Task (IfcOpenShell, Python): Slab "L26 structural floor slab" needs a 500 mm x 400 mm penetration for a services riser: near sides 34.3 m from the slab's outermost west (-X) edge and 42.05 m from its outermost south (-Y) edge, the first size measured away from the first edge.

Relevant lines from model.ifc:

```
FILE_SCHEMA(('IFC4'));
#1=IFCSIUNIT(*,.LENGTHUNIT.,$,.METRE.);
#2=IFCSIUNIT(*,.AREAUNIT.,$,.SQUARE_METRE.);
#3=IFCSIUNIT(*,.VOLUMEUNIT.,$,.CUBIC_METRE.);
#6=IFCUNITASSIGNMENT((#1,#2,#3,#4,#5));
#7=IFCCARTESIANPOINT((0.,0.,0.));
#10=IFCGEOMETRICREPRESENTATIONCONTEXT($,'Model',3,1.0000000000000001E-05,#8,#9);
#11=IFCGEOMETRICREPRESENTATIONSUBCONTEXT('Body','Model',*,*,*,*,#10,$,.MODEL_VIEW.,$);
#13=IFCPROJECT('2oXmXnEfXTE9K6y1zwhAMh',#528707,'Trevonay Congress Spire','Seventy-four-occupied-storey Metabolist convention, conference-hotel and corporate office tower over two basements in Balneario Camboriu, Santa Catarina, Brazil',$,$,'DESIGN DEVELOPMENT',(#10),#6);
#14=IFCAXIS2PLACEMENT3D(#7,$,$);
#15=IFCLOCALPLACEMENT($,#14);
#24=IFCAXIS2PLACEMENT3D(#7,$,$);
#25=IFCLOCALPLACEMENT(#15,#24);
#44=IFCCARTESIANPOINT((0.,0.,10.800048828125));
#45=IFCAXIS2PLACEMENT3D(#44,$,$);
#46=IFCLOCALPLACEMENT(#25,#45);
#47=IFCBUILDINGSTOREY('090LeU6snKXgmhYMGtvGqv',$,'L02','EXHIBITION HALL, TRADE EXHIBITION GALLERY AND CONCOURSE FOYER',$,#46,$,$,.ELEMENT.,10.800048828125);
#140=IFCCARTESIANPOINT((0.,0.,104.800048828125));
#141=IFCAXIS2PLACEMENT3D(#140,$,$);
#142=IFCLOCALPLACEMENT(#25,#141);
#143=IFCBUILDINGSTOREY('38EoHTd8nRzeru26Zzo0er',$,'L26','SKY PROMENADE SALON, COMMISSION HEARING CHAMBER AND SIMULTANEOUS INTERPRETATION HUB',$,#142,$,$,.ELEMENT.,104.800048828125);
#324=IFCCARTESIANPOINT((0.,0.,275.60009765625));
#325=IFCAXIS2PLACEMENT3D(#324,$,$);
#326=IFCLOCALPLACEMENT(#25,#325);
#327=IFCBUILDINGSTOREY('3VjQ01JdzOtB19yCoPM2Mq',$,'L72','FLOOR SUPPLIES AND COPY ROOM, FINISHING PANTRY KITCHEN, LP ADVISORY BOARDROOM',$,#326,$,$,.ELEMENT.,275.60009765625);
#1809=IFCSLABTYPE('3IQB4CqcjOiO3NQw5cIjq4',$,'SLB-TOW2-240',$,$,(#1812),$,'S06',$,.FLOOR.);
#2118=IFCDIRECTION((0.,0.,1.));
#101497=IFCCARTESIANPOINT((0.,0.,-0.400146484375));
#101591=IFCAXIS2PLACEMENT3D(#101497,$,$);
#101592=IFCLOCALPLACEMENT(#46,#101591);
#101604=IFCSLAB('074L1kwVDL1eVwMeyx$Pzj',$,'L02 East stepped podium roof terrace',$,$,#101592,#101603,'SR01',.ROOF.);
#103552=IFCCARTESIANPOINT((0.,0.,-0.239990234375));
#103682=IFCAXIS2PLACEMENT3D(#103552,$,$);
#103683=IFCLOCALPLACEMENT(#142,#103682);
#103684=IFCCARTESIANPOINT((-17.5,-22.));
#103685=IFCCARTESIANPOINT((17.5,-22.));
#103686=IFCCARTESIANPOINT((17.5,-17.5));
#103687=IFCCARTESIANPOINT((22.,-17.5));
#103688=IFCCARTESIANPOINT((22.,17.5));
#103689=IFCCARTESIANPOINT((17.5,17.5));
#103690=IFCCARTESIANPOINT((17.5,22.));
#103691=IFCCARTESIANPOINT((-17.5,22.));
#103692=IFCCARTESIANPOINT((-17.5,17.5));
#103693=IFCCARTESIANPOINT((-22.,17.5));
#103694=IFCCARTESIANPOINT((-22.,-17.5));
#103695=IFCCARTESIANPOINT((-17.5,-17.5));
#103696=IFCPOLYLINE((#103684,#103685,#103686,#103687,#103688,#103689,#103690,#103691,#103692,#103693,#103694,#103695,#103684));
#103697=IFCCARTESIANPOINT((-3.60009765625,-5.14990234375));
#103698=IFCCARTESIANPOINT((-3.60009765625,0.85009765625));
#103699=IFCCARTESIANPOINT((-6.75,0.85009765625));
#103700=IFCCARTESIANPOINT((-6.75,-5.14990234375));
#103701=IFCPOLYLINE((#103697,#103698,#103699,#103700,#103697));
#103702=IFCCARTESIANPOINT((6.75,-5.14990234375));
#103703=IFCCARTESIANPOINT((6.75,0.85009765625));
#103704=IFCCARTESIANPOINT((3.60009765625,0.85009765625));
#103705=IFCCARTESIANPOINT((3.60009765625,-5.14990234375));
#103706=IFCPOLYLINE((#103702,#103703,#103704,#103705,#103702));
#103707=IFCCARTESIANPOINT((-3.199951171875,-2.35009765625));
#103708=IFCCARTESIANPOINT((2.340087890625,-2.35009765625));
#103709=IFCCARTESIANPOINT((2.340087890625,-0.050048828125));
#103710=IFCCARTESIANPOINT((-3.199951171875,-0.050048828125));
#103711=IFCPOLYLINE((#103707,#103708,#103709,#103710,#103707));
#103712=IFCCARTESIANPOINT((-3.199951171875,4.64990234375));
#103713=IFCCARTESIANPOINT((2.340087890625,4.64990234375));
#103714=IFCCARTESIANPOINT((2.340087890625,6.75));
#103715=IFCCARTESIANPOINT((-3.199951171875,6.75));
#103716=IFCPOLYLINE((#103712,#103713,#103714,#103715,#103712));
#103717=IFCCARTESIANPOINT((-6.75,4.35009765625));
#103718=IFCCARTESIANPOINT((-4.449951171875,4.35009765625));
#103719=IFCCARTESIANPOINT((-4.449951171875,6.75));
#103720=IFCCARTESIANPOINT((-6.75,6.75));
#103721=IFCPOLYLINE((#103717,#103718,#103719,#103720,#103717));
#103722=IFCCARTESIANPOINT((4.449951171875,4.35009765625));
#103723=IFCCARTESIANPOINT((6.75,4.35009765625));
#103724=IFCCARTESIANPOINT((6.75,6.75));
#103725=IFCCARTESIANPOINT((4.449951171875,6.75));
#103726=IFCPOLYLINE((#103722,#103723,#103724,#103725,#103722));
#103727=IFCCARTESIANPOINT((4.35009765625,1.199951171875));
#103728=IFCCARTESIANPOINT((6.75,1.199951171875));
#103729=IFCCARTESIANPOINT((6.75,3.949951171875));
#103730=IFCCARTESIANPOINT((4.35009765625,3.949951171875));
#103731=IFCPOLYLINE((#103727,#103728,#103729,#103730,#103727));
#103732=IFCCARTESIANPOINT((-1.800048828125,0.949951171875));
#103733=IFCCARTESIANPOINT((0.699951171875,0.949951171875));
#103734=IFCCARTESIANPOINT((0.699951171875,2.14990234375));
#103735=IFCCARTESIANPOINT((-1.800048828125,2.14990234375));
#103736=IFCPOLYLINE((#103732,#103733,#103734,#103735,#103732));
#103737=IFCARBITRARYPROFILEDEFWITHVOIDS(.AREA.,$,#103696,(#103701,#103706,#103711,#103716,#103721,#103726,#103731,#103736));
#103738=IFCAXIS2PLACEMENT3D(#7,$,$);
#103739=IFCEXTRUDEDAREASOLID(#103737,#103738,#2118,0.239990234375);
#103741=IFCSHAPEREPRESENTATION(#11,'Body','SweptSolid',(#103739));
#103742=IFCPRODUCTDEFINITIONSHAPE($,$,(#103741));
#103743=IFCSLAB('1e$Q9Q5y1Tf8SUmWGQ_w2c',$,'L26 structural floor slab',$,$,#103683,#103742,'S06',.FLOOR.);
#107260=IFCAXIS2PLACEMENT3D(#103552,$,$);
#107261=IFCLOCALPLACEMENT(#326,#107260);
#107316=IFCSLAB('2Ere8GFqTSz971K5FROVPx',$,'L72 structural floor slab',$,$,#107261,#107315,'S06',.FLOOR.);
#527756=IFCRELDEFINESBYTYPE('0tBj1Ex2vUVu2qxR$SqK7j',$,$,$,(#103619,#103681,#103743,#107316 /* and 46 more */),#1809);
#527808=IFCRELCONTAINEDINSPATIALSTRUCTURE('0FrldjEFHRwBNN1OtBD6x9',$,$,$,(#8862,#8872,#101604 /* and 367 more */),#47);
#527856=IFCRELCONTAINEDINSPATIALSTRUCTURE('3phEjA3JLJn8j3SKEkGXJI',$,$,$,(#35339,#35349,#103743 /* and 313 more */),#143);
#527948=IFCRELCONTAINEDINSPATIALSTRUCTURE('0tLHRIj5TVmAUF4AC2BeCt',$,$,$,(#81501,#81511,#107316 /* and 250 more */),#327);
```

```python
import numpy as np
import ifcopenshell
import ifcopenshell.api.feature
import ifcopenshell.api.geometry
import ifcopenshell.api.root
import ifcopenshell.geom
import ifcopenshell.util.placement
import ifcopenshell.util.representation
import ifcopenshell.util.shape
import ifcopenshell.util.unit

model = ifcopenshell.open("model.ifc")
unit_scale = ifcopenshell.util.unit.calculate_unit_scale(model)
settings = ifcopenshell.geom.settings()


def volume(element):
    """Net volume in cubic metres, openings subtracted."""
    shape = ifcopenshell.geom.create_shape(settings, element)
    return ifcopenshell.util.shape.get_volume(shape.geometry)


slab = model.by_guid("1e$Q9Q5y1Tf8SUmWGQ_w2c")
before = volume(slab)

# Extent in the slab's own axes, in metres. The edges named are its -X and -Y sides.
slab_shape = ifcopenshell.geom.create_shape(settings, slab)
vertices = ifcopenshell.util.shape.get_vertices(slab_shape.geometry)
x_min, y_min, bottom = vertices.min(axis=0)
top = vertices[:, 2].max()

opening = ifcopenshell.api.root.create_entity(model, ifc_class="IfcOpeningElement", name="Services riser opening", predefined_type="OPENING")
context = ifcopenshell.util.representation.get_context(model, "Model", "Body", "MODEL_VIEW")
width, depth = 0.5, 0.4
outline = [(0.0, 0.0), (width, 0.0), (width, depth), (0.0, depth), (0.0, 0.0)]
# Overshoot both faces by 50 mm so the cut is clean.
shape = ifcopenshell.api.geometry.add_slab_representation(
    model, context=context, depth=top - bottom + 0.1, polyline=outline
)
ifcopenshell.api.geometry.assign_representation(model, product=opening, representation=shape)

matrix = ifcopenshell.util.placement.get_local_placement(slab.ObjectPlacement)
matrix[:, 3] = matrix @ np.append(np.array([x_min + 34.3, y_min + 42.05, bottom - 0.05]) / unit_scale, 1.0)
ifcopenshell.api.geometry.edit_object_placement(model, product=opening, matrix=matrix, is_si=False)
ifcopenshell.api.feature.add_feature(model, feature=opening, element=slab)

after = volume(slab)

print(f"slab volume {before:.3f} -> {after:.3f} m3")

model.write("model_edited.ifc")
```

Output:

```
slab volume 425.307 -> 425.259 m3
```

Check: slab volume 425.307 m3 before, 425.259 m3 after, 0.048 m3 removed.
